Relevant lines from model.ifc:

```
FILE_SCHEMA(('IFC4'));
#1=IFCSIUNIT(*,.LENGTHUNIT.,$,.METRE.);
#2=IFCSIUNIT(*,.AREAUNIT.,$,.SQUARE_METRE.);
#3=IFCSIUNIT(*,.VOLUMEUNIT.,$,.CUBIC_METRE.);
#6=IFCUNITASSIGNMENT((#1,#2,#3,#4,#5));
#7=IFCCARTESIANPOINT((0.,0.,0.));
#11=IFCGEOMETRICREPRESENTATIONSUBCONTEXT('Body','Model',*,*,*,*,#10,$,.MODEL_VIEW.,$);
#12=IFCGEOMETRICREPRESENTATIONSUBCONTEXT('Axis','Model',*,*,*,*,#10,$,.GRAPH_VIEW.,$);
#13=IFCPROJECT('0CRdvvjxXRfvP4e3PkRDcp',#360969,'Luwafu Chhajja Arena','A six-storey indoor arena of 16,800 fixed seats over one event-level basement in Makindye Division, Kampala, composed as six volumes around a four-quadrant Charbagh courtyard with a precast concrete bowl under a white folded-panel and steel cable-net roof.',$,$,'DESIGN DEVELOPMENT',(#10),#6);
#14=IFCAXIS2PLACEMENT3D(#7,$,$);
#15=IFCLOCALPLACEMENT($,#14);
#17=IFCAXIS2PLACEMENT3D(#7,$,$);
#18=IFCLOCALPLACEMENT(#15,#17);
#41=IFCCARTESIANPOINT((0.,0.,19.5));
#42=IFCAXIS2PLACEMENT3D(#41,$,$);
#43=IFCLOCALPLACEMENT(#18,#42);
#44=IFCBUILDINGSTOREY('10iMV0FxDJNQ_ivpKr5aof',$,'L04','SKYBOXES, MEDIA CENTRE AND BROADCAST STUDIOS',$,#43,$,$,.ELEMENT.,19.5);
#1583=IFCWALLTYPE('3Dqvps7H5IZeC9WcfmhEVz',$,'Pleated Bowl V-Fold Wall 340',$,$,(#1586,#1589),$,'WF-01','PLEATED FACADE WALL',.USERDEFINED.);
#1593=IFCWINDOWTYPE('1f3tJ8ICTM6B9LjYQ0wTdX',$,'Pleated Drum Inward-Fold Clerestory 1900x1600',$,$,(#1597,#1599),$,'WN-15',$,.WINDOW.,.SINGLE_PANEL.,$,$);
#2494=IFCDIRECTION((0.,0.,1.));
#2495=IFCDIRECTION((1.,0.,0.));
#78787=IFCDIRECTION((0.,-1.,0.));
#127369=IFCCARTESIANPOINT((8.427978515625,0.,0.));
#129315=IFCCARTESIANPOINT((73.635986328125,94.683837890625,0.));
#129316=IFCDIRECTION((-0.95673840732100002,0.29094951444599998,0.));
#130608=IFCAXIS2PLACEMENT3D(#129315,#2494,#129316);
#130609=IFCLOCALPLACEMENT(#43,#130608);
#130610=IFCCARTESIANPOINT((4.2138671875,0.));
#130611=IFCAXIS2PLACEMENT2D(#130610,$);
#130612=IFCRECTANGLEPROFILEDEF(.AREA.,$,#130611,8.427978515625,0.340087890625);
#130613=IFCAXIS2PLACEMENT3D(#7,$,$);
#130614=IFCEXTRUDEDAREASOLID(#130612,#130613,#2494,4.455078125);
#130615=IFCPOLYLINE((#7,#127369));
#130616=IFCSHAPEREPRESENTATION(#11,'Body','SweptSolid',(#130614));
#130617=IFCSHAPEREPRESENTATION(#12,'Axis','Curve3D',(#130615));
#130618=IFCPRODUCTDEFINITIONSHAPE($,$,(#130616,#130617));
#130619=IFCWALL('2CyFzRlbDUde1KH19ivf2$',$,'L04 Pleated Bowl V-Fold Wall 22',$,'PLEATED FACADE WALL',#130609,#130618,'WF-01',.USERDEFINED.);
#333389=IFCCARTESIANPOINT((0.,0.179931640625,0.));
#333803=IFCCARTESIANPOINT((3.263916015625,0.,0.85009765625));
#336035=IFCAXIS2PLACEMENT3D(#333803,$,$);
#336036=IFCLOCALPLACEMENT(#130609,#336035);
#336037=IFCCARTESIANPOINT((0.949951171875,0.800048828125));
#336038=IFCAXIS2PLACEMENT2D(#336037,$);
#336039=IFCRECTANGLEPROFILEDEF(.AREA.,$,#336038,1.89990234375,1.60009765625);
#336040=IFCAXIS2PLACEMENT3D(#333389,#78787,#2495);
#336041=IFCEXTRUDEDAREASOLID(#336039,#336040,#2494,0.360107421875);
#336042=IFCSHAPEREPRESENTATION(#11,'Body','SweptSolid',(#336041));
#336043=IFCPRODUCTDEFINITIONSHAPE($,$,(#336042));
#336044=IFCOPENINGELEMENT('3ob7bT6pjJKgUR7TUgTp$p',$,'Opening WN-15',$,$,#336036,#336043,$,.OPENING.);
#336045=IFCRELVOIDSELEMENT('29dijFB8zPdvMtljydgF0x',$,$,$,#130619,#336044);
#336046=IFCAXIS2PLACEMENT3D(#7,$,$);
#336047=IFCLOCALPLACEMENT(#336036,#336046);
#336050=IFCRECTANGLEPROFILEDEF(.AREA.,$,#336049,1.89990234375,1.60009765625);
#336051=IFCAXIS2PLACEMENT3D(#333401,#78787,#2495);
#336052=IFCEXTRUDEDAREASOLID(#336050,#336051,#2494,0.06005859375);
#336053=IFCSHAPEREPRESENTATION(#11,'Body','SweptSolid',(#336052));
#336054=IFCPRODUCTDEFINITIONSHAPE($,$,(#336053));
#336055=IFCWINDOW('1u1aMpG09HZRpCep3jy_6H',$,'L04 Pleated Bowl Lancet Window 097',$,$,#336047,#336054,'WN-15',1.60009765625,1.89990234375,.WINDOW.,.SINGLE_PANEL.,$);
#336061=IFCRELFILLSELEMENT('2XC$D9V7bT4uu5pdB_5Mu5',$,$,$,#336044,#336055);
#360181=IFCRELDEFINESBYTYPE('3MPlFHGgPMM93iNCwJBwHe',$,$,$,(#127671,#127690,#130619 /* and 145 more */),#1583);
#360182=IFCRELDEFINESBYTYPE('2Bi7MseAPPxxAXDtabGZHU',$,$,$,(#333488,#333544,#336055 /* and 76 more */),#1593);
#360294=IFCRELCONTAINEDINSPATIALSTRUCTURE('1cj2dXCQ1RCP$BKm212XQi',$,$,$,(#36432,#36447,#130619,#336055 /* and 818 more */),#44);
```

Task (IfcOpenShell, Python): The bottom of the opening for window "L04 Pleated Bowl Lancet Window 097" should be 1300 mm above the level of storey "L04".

```python
import numpy as np
import ifcopenshell
import ifcopenshell.api.geometry
import ifcopenshell.geom
import ifcopenshell.util.element
import ifcopenshell.util.placement
import ifcopenshell.util.shape
import ifcopenshell.util.unit

model = ifcopenshell.open("model.ifc")
unit_scale = ifcopenshell.util.unit.calculate_unit_scale(model)

window = model.by_guid("1u1aMpG09HZRpCep3jy_6H")
opening = window.FillsVoids[0].RelatingOpeningElement
storey = ifcopenshell.util.element.get_container(window, ifc_class="IfcBuildingStorey")
level = ifcopenshell.util.placement.get_local_placement(storey.ObjectPlacement)[2, 3]

# The opening's origin need not be at the sill, so measure its lowest point.
shape = ifcopenshell.geom.create_shape(ifcopenshell.geom.settings(), opening)
bottom = ifcopenshell.util.shape.get_shape_bottom_elevation(shape, shape.geometry) / unit_scale
dz = level + 1.3 / unit_scale - bottom

shift = np.array([0.0, 0.0, dz])
# The window is placed relative to its opening, so it follows when the opening moves.
matrix = ifcopenshell.util.placement.get_local_placement(opening.ObjectPlacement)
matrix[:3, 3] += shift
ifcopenshell.api.geometry.edit_object_placement(
    model, product=opening, matrix=matrix, is_si=False, should_transform_children=True
)

print(f"moved by {dz * unit_scale:+.3f} m")

model.write("model_v2.ifc")
```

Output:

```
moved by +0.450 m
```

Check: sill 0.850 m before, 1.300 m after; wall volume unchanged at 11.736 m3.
